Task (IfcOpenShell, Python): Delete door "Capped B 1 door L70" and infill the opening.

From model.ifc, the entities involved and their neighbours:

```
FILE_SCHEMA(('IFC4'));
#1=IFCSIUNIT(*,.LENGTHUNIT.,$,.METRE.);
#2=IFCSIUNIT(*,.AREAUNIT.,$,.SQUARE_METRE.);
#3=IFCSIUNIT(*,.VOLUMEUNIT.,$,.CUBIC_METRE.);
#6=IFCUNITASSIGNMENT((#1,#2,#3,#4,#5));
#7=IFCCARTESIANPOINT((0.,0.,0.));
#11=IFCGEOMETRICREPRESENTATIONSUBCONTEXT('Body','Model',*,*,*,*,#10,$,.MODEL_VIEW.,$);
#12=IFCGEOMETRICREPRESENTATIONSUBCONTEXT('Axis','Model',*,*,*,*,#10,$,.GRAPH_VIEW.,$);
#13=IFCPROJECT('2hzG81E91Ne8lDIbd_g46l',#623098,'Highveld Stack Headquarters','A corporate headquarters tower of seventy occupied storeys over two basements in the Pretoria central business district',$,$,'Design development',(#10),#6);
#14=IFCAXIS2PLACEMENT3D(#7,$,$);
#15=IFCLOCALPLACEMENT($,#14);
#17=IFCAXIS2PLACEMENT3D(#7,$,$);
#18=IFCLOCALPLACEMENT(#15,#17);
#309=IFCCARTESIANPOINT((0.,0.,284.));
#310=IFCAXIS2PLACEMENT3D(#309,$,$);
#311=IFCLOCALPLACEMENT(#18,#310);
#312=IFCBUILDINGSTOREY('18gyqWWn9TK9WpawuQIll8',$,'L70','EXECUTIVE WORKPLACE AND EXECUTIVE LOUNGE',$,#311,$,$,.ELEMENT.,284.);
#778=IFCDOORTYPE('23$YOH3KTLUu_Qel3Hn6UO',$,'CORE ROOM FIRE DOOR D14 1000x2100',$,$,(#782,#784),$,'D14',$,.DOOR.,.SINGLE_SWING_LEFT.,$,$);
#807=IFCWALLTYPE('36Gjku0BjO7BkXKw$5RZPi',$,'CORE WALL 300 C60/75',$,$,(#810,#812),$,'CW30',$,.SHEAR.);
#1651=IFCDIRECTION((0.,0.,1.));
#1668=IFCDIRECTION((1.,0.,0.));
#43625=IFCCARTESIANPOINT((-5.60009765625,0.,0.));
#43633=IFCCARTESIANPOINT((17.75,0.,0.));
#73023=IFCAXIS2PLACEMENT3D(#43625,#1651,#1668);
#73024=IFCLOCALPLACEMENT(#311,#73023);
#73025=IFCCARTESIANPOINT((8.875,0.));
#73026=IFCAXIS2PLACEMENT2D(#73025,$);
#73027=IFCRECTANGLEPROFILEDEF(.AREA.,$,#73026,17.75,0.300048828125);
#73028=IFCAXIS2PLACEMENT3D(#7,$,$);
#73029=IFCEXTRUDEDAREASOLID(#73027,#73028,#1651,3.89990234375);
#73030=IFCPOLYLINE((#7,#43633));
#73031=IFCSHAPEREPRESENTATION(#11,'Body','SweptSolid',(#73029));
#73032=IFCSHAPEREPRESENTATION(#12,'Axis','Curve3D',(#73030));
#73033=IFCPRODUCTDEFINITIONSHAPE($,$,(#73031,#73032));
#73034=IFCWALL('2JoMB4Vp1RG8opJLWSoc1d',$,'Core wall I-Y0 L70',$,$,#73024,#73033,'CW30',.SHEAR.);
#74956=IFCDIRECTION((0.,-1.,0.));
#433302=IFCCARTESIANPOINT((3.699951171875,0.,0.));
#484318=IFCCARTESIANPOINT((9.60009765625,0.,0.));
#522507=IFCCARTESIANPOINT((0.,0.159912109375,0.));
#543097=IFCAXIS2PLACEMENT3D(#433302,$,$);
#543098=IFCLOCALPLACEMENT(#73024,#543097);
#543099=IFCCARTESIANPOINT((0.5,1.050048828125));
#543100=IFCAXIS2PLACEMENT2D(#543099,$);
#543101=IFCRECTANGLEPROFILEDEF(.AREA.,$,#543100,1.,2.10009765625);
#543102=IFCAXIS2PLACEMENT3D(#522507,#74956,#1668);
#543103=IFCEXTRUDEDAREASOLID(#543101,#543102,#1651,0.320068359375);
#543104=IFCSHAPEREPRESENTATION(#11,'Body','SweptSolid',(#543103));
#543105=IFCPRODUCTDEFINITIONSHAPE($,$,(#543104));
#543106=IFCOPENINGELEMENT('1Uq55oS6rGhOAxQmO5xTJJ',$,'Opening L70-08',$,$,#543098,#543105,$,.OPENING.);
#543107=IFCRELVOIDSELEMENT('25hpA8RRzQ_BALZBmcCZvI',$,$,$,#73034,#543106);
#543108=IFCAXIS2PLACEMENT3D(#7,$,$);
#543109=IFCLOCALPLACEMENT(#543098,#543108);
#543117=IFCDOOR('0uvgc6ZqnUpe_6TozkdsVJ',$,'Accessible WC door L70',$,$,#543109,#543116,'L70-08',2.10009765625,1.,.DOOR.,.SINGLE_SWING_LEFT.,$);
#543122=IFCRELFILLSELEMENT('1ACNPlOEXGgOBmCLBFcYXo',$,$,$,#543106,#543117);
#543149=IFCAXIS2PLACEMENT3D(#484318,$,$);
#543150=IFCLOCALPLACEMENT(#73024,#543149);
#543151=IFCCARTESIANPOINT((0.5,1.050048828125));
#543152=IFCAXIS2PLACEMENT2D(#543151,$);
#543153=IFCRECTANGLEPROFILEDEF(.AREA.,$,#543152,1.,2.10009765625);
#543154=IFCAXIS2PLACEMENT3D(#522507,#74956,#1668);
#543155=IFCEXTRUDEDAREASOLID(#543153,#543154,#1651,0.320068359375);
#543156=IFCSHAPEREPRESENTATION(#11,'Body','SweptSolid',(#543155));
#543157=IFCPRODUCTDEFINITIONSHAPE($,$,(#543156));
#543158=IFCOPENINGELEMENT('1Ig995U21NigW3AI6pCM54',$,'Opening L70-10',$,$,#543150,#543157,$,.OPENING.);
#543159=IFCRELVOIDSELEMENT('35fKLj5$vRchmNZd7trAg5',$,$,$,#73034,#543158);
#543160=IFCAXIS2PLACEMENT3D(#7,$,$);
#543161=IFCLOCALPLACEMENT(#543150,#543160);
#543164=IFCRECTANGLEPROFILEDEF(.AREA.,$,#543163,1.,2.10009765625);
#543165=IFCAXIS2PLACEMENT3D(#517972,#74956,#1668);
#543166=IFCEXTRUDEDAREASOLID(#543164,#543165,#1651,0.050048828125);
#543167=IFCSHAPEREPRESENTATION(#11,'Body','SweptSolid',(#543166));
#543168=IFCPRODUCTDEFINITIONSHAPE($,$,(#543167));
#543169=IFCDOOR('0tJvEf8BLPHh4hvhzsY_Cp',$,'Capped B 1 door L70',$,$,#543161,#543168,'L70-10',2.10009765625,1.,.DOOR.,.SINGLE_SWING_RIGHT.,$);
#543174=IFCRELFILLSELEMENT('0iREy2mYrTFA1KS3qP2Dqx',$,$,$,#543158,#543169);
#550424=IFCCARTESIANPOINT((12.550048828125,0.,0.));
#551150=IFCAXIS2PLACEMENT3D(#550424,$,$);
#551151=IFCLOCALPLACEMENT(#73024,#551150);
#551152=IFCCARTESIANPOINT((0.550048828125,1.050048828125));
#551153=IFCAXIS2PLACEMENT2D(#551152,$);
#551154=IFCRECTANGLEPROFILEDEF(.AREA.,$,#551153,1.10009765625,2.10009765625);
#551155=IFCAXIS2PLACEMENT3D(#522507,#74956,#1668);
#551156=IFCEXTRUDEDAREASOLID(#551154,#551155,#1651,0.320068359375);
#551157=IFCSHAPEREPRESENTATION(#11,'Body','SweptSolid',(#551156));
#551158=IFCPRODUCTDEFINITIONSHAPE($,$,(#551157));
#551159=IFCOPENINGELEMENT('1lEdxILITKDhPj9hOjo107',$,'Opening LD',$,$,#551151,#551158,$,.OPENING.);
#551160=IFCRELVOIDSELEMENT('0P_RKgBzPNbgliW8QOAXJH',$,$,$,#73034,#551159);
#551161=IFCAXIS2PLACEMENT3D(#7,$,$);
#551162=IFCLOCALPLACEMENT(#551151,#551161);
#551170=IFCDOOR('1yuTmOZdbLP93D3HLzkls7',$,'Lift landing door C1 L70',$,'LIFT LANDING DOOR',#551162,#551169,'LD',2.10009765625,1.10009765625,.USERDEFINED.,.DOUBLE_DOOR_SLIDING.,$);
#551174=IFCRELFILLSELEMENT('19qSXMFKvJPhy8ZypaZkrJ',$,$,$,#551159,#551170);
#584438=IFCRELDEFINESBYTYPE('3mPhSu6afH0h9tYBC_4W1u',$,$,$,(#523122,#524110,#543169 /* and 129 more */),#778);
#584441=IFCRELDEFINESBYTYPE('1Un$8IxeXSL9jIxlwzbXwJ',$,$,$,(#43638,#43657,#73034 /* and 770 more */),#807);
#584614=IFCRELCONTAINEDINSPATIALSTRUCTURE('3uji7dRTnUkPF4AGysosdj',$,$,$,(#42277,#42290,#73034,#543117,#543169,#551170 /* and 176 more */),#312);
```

```python
import ifcopenshell
import ifcopenshell.api.feature
import ifcopenshell.api.root
import ifcopenshell.geom
import ifcopenshell.util.shape

model = ifcopenshell.open("model.ifc")
settings = ifcopenshell.geom.settings()


def volume(element):
    """Net volume in cubic metres, openings subtracted."""
    shape = ifcopenshell.geom.create_shape(settings, element)
    return ifcopenshell.util.shape.get_volume(shape.geometry)


door = model.by_guid("0tJvEf8BLPHh4hvhzsY_Cp")
opening = door.FillsVoids[0].RelatingOpeningElement
wall = opening.VoidsElements[0].RelatingBuildingElement
before = volume(wall)

ifcopenshell.api.root.remove_product(model, product=door)
ifcopenshell.api.feature.remove_feature(model, feature=opening)

after = volume(wall)

print(f"wall volume {before:.3f} -> {after:.3f} m3")

model.write("model_v2.ifc")
```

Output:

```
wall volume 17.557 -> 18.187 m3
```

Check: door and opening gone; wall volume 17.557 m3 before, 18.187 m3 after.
